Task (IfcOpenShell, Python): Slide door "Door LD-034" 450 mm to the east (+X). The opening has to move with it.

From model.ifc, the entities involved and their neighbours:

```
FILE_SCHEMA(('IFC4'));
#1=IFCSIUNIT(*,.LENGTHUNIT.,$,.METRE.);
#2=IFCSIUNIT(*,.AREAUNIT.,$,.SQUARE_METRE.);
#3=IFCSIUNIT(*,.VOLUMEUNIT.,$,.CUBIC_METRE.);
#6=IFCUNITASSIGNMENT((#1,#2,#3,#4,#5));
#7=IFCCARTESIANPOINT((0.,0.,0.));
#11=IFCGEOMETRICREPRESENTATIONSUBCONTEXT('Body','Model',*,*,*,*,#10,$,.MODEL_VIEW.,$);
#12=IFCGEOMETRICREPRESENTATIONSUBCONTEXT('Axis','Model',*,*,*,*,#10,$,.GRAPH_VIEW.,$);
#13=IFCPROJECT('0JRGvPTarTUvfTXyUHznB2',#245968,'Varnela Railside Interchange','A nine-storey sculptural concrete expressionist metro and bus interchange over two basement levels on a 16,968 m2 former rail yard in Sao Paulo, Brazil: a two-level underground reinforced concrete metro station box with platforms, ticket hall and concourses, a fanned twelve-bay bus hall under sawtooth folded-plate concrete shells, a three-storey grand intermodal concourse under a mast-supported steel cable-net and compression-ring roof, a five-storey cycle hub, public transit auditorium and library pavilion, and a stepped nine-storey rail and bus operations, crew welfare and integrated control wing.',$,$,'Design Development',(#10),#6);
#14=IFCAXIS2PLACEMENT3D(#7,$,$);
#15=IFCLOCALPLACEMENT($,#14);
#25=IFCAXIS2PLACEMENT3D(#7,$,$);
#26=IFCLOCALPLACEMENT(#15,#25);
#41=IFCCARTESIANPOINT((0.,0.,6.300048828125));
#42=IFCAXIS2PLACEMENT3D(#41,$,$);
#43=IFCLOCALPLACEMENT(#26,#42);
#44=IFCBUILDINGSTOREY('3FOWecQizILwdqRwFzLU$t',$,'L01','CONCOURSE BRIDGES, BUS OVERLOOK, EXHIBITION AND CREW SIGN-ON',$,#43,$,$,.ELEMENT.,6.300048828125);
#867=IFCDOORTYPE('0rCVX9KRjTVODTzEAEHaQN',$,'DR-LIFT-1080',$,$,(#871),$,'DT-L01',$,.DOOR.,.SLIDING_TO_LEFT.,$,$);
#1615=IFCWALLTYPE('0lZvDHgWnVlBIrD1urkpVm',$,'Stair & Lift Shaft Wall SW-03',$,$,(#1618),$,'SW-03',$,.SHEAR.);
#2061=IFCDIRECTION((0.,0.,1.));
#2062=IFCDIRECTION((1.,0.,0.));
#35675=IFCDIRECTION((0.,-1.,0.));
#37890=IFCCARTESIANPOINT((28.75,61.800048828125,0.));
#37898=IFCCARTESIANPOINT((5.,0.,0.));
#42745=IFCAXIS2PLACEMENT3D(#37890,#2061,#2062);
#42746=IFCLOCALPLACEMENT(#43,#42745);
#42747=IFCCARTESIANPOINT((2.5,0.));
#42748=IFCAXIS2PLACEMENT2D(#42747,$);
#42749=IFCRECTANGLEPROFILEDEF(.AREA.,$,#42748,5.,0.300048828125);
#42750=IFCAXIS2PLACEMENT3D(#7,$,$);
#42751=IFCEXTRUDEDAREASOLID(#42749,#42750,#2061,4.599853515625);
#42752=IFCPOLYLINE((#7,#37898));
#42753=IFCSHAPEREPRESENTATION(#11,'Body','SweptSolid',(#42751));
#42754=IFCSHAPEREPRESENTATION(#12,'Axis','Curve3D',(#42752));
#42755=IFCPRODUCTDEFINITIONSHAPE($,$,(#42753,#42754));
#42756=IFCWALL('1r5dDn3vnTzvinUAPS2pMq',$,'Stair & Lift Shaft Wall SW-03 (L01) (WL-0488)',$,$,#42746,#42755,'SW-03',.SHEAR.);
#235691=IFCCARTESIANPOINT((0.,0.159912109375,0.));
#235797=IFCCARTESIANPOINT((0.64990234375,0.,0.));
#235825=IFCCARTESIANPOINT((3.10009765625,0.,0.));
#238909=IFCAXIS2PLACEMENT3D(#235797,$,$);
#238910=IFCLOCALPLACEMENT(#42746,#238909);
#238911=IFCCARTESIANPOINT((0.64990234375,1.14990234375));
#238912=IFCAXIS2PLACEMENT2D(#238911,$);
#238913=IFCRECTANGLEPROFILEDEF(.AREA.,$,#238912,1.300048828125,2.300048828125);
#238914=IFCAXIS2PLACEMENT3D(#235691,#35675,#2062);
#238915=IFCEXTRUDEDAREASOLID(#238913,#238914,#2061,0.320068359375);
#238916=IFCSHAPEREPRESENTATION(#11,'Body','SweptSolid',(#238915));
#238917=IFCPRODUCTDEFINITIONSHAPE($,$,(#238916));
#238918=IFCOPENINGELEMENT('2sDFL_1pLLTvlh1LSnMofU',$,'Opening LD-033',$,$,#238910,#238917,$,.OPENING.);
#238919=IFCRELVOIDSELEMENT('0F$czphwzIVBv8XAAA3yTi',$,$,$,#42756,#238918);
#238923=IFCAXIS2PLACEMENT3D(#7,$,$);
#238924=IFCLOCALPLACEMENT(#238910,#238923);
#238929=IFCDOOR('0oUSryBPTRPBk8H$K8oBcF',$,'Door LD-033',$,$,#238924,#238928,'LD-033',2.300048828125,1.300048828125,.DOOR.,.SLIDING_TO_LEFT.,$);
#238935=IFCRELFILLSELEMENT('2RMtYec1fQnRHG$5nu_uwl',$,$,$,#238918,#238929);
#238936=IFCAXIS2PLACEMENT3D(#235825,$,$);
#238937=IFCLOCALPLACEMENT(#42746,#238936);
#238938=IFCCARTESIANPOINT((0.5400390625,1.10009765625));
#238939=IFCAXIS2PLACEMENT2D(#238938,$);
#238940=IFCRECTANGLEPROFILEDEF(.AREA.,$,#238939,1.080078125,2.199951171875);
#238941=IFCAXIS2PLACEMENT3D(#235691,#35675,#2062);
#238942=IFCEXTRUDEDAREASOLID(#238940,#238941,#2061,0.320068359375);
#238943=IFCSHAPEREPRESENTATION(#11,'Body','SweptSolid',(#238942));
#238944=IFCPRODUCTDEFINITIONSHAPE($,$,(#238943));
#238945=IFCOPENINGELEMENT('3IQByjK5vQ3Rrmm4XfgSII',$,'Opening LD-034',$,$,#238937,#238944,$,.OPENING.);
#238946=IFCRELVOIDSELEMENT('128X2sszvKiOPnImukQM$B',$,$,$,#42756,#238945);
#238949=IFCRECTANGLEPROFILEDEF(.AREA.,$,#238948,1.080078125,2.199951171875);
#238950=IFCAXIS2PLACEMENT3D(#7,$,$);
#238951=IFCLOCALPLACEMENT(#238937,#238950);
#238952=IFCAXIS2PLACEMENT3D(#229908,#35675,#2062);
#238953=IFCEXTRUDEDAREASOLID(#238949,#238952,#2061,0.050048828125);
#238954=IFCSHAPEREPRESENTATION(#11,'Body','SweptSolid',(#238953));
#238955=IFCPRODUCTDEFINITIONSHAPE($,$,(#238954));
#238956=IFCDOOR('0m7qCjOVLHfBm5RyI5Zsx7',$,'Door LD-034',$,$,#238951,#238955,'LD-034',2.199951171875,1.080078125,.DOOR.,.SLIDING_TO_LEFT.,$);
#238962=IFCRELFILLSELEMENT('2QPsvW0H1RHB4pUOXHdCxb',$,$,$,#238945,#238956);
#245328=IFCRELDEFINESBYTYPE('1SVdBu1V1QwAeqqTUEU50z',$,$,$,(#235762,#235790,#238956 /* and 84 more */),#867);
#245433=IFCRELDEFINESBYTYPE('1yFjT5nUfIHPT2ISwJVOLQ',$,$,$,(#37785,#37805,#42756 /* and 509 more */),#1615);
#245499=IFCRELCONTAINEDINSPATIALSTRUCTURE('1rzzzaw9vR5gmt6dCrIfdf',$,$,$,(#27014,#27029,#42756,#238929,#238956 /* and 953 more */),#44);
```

```python
import ifcopenshell
import ifcopenshell.api.geometry
import ifcopenshell.util.placement
import ifcopenshell.util.unit

model = ifcopenshell.open("model.ifc")
unit_scale = ifcopenshell.util.unit.calculate_unit_scale(model)

door = model.by_id(238956)
opening = door.FillsVoids[0].RelatingOpeningElement
wall = opening.VoidsElements[0].RelatingBuildingElement

wall_matrix = ifcopenshell.util.placement.get_local_placement(wall.ObjectPlacement)
shift = wall_matrix[:3, 0] * 0.45 / unit_scale
before = ifcopenshell.util.placement.get_local_placement(door.ObjectPlacement)[:3, 3].copy()

# The door is placed relative to its opening, so it follows when the opening moves.
matrix = ifcopenshell.util.placement.get_local_placement(opening.ObjectPlacement)
matrix[:3, 3] += shift
ifcopenshell.api.geometry.edit_object_placement(
    model, product=opening, matrix=matrix, is_si=False, should_transform_children=True
)

after = ifcopenshell.util.placement.get_local_placement(door.ObjectPlacement)[:3, 3]
print("door moved by", (after - before).round(3) + 0.0)

model.write("model-out.ifc")
```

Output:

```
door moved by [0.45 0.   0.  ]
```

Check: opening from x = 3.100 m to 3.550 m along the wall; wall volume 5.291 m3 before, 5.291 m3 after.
